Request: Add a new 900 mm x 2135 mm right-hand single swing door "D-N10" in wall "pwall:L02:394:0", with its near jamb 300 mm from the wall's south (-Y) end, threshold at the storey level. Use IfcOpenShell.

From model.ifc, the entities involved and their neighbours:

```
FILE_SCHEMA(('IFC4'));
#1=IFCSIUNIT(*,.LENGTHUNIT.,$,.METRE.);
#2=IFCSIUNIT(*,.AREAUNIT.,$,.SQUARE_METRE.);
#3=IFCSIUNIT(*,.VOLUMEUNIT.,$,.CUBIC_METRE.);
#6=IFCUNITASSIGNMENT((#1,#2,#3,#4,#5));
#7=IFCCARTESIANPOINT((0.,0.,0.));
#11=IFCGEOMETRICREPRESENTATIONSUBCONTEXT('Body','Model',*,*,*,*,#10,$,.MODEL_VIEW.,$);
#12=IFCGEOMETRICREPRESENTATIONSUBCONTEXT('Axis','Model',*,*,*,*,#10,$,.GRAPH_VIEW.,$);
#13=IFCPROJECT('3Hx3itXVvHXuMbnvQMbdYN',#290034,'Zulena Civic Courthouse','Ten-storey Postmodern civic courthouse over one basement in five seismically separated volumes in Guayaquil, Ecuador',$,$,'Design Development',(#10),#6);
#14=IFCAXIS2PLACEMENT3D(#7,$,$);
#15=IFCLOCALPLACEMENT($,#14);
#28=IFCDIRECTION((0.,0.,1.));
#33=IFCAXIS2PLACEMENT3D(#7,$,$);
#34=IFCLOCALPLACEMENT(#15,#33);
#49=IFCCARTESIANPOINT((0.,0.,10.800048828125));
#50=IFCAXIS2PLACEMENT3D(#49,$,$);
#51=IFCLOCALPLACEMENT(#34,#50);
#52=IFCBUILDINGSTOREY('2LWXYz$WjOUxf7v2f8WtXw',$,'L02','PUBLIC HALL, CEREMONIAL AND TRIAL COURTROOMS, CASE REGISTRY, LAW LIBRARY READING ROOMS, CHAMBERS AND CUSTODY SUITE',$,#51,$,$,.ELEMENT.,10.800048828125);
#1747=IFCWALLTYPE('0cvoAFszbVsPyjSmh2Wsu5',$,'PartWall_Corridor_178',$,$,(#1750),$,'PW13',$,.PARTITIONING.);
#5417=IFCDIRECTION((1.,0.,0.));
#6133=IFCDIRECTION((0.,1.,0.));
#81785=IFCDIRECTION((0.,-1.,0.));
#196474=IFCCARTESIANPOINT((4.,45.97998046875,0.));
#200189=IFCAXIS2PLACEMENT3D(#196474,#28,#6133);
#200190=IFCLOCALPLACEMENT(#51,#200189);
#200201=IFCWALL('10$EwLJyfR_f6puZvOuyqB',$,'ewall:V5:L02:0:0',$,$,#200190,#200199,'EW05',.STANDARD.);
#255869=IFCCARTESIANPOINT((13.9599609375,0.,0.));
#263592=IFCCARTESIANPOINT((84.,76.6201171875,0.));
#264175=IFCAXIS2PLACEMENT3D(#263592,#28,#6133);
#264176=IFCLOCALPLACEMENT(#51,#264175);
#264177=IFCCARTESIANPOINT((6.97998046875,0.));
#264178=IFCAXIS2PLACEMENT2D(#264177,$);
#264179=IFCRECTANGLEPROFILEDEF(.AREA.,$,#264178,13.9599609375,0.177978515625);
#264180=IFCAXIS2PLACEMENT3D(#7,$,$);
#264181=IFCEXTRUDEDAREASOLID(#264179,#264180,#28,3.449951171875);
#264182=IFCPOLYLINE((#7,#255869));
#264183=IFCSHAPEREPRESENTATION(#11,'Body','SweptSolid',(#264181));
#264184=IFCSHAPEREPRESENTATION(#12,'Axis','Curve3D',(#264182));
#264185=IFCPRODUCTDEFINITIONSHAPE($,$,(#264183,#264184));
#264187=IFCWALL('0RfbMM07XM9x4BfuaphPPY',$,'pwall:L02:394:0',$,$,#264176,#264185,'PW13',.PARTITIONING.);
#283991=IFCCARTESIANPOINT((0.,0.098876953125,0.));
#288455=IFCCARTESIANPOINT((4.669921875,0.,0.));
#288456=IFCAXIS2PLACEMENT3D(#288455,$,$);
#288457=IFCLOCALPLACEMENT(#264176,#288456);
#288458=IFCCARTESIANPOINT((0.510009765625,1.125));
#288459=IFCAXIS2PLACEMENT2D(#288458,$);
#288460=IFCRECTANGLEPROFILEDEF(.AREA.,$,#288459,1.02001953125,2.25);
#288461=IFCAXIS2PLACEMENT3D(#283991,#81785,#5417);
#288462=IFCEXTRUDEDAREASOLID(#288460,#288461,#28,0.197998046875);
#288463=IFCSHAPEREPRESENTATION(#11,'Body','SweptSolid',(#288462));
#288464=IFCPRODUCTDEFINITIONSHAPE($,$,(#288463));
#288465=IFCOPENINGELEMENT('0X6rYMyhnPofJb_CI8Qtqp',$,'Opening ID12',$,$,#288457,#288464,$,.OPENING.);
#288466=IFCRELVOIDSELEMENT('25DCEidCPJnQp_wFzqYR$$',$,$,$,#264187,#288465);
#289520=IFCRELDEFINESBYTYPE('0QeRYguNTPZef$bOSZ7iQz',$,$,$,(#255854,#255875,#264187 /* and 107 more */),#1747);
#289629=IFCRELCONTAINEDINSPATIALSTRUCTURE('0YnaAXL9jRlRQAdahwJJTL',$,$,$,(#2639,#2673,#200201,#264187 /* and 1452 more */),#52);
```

```python
import numpy as np
import ifcopenshell
import ifcopenshell.api.feature
import ifcopenshell.api.geometry
import ifcopenshell.api.root
import ifcopenshell.api.spatial
import ifcopenshell.geom
import ifcopenshell.util.element
import ifcopenshell.util.placement
import ifcopenshell.util.representation
import ifcopenshell.util.shape
import ifcopenshell.util.unit

model = ifcopenshell.open("model.ifc")
unit_scale = ifcopenshell.util.unit.calculate_unit_scale(model)
settings = ifcopenshell.geom.settings()


def volume(element):
    """Net volume in cubic metres, openings subtracted."""
    shape = ifcopenshell.geom.create_shape(settings, element)
    return ifcopenshell.util.shape.get_volume(shape.geometry)


wall = model.by_id(264187)
storey = ifcopenshell.util.element.get_container(wall, ifc_class="IfcBuildingStorey")
context = ifcopenshell.util.representation.get_context(model, "Model", "Body", "MODEL_VIEW")
before = volume(wall)

width, height, from_end, sill = 0.9, 2.135, 0.3, 0.0  # metres

# The wall runs along its own X axis, and the end named is its -X end.
wall_shape = ifcopenshell.geom.create_shape(settings, wall)
x, y, z = ifcopenshell.util.shape.get_vertices(wall_shape.geometry).T
start = x.min() + from_end
face, thickness = float(y.min()), float(y.max() - y.min())
wall_matrix = ifcopenshell.util.placement.get_local_placement(wall.ObjectPlacement)
level = ifcopenshell.util.placement.get_local_placement(storey.ObjectPlacement)[2, 3]


def in_wall(x, y):
    """Placement at x, y metres in the wall's axes, at sill height."""
    matrix = wall_matrix.copy()
    matrix[:, 3] = wall_matrix @ np.array([x / unit_scale, y / unit_scale, 0.0, 1.0])
    matrix[2, 3] = level + sill / unit_scale
    return matrix


# Opening: a box that overshoots both wall faces by 50 mm.
opening = ifcopenshell.api.root.create_entity(model, ifc_class="IfcOpeningElement", predefined_type="OPENING")
box = ifcopenshell.api.geometry.add_wall_representation(
    model, context=context, length=width, height=height, thickness=thickness + 0.1
)
ifcopenshell.api.geometry.assign_representation(model, product=opening, representation=box)
ifcopenshell.api.geometry.edit_object_placement(model, product=opening, matrix=in_wall(start, face - 0.05), is_si=False)
ifcopenshell.api.feature.add_feature(model, feature=opening, element=wall)

door = ifcopenshell.api.root.create_entity(model, ifc_class="IfcDoor", name="D-N10", predefined_type="DOOR")
door.OverallWidth, door.OverallHeight = width / unit_scale, height / unit_scale
door.OperationType = "SINGLE_SWING_RIGHT"
body = ifcopenshell.api.geometry.add_door_representation(
    model,
    context=context,
    overall_width=door.OverallWidth,
    overall_height=door.OverallHeight,
    operation_type="SINGLE_SWING_RIGHT",
    lining_properties={"LiningDepth": thickness / unit_scale, "ThresholdDepth": thickness / unit_scale},
)
ifcopenshell.api.geometry.assign_representation(model, product=door, representation=body)
ifcopenshell.api.spatial.assign_container(model, products=[door], relating_structure=storey)
ifcopenshell.api.feature.add_filling(model, opening=opening, element=door)

# The lining spans the wall, so the door starts at the wall face.
ifcopenshell.api.geometry.edit_object_placement(model, product=door, matrix=in_wall(start, face), is_si=False)

after = volume(wall)

print(f"wall volume {before:.3f} -> {after:.3f} m3")

model.write("model_edited.ifc")
```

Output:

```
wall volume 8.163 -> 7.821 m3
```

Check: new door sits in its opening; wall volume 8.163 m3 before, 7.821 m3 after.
